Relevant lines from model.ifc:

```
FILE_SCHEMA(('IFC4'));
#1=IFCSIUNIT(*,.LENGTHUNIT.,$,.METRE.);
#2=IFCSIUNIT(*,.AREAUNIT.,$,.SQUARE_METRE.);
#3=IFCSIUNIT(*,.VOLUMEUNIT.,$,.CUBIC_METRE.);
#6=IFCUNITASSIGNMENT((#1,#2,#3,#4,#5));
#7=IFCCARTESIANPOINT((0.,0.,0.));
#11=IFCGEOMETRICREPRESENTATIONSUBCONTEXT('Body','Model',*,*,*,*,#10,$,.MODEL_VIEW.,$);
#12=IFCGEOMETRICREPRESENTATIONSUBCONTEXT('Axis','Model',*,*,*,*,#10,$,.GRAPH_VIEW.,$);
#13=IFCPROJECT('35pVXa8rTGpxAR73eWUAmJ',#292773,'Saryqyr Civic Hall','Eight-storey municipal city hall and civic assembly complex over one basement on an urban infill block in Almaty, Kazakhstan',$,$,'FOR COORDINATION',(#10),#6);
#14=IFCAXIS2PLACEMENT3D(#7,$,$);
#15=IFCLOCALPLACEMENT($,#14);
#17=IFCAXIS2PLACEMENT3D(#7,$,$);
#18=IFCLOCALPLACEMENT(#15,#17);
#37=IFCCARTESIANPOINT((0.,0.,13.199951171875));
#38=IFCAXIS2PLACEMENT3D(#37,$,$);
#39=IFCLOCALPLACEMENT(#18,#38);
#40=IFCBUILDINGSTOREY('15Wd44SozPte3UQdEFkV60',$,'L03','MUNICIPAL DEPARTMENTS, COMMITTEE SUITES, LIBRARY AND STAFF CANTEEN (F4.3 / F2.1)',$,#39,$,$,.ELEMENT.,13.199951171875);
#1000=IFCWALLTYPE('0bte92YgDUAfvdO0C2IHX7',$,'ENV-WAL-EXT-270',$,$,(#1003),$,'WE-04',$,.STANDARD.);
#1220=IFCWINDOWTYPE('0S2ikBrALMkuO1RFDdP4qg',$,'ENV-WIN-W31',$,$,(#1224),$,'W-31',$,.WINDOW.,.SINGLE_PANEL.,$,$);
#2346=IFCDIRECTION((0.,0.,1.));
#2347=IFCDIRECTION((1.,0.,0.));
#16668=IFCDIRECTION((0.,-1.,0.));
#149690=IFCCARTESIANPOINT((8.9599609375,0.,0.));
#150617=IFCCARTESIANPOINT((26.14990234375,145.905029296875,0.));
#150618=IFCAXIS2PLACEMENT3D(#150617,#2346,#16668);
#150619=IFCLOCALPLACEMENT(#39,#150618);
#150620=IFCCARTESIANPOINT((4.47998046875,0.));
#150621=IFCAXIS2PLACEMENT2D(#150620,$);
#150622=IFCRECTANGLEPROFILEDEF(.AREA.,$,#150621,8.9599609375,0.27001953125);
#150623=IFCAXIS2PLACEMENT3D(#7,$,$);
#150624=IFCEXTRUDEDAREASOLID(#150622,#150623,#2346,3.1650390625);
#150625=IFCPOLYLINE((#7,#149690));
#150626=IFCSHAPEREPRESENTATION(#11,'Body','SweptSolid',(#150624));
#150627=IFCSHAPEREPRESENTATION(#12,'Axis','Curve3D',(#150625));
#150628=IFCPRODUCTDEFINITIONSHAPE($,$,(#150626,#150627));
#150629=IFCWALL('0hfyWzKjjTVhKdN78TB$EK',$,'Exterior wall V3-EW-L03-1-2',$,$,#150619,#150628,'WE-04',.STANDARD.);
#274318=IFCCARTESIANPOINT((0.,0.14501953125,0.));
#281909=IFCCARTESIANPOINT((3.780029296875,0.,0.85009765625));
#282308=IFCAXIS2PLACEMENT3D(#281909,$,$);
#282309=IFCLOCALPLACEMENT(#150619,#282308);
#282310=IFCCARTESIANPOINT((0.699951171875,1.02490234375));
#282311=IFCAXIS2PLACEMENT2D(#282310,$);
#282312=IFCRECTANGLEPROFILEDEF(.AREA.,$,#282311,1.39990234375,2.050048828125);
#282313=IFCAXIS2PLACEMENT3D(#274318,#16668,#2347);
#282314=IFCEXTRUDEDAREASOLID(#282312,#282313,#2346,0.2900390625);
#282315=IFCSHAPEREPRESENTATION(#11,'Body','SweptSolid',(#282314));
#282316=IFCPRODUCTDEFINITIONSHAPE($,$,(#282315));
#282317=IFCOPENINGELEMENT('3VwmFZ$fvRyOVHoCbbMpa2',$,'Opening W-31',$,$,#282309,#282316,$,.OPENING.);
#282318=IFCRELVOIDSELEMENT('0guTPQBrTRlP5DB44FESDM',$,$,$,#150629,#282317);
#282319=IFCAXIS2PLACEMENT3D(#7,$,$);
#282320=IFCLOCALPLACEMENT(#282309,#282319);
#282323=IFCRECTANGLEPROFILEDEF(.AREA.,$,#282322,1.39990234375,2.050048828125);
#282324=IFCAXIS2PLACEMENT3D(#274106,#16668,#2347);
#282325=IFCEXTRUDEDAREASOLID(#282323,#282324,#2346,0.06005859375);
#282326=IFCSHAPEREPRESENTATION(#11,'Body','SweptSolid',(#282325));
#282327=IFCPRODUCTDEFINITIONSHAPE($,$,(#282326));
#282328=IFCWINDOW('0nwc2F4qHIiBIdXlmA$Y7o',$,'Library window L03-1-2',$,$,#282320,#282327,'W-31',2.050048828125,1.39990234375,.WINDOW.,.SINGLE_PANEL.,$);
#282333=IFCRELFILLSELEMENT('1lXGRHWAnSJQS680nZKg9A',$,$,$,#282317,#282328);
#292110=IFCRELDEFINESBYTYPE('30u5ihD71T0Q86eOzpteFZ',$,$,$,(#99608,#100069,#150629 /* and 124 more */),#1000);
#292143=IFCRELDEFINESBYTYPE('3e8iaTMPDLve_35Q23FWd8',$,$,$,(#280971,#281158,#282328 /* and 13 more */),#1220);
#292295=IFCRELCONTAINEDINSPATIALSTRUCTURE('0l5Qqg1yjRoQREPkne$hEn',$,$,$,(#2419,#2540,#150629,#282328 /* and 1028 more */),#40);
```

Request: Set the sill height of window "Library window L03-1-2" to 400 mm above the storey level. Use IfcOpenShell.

```python
import numpy as np
import ifcopenshell
import ifcopenshell.api.geometry
import ifcopenshell.geom
import ifcopenshell.util.element
import ifcopenshell.util.placement
import ifcopenshell.util.shape
import ifcopenshell.util.unit

model = ifcopenshell.open("model.ifc")
unit_scale = ifcopenshell.util.unit.calculate_unit_scale(model)

window = model.by_guid("0nwc2F4qHIiBIdXlmA$Y7o")
opening = window.FillsVoids[0].RelatingOpeningElement
storey = ifcopenshell.util.element.get_container(window, ifc_class="IfcBuildingStorey")
level = ifcopenshell.util.placement.get_local_placement(storey.ObjectPlacement)[2, 3]

# The opening's origin need not be at the sill, so measure its lowest point.
shape = ifcopenshell.geom.create_shape(ifcopenshell.geom.settings(), opening)
bottom = ifcopenshell.util.shape.get_shape_bottom_elevation(shape, shape.geometry) / unit_scale
dz = level + 0.4 / unit_scale - bottom

shift = np.array([0.0, 0.0, dz])
# The window is placed relative to its opening, so it follows when the opening moves.
matrix = ifcopenshell.util.placement.get_local_placement(opening.ObjectPlacement)
matrix[:3, 3] += shift
ifcopenshell.api.geometry.edit_object_placement(
    model, product=opening, matrix=matrix, is_si=False, should_transform_children=True
)

print(f"moved by {dz * unit_scale:+.3f} m")

model.write("model_edited.ifc")
```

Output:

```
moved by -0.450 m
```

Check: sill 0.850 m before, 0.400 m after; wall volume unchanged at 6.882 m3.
